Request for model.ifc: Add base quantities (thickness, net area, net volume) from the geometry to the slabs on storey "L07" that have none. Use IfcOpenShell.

First a look at what the model holds.

```python
import ifcopenshell
import ifcopenshell.util.element
import ifcopenshell.util.unit

model = ifcopenshell.open("model.ifc")
print(model.schema)
for unit_type in ("LENGTHUNIT", "AREAUNIT", "VOLUMEUNIT"):
    print(unit_type, ifcopenshell.util.unit.calculate_unit_scale(model, unit_type))
storey = next(s for s in model.by_type("IfcBuildingStorey") if s.Name == "L07")
slabs = [e for e in ifcopenshell.util.element.get_decomposition(storey) if e.is_a("IfcSlab")]
for e in sorted(slabs, key=lambda e: e.id()):
    print(e.id(), e.is_a(), e.Name, list(ifcopenshell.util.element.get_psets(e, qtos_only=True)), sep=" | ")
```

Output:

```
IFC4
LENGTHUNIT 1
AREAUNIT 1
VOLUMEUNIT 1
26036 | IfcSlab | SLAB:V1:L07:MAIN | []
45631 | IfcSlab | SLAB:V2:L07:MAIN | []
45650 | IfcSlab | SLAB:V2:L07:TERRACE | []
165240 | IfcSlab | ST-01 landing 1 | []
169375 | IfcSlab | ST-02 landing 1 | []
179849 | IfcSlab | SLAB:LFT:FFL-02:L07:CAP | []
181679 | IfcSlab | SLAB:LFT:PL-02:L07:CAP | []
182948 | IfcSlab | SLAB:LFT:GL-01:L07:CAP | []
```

```python
import ifcopenshell
import ifcopenshell.api.pset
import ifcopenshell.geom
import ifcopenshell.util.element
import ifcopenshell.util.shape
import ifcopenshell.util.unit

model = ifcopenshell.open("model.ifc")
unit_scale = ifcopenshell.util.unit.calculate_unit_scale(model)
area_scale = ifcopenshell.util.unit.calculate_unit_scale(model, "AREAUNIT")
volume_scale = ifcopenshell.util.unit.calculate_unit_scale(model, "VOLUMEUNIT")
settings = ifcopenshell.geom.settings()

storey = next(s for s in model.by_type("IfcBuildingStorey") if s.Name == "L07")
slabs = [e for e in ifcopenshell.util.element.get_decomposition(storey) if e.is_a("IfcSlab")]

for e in sorted(slabs, key=lambda e: e.id()):
    if ifcopenshell.util.element.get_psets(e, qtos_only=True, should_inherit=False):
        continue
    # Geometry comes back in metres, in the element's own axes.
    shape = ifcopenshell.geom.create_shape(settings, e)
    values = {
        "Width": ifcopenshell.util.shape.get_z(shape.geometry) / unit_scale,
        "NetArea": ifcopenshell.util.shape.get_footprint_area(shape.geometry) / area_scale,
        "NetVolume": ifcopenshell.util.shape.get_volume(shape.geometry) / volume_scale,
    }
    qto = ifcopenshell.api.pset.add_qto(model, product=e, name="Qto_SlabBaseQuantities")
    ifcopenshell.api.pset.edit_qto(model, qto=qto, properties=values)
    print(e.id(), {k: round(v, 3) for k, v in values.items()})

model.write("model-out.ifc")
```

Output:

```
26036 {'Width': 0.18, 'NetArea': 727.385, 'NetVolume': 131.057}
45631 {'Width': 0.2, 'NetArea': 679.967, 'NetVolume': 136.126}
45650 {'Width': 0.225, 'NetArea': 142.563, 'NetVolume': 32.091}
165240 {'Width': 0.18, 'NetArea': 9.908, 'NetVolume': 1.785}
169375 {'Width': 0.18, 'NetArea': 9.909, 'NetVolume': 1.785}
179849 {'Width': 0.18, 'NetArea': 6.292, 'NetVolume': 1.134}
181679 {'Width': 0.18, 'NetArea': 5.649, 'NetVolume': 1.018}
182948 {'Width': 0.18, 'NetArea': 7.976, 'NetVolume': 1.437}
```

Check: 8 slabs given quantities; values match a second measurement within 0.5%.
